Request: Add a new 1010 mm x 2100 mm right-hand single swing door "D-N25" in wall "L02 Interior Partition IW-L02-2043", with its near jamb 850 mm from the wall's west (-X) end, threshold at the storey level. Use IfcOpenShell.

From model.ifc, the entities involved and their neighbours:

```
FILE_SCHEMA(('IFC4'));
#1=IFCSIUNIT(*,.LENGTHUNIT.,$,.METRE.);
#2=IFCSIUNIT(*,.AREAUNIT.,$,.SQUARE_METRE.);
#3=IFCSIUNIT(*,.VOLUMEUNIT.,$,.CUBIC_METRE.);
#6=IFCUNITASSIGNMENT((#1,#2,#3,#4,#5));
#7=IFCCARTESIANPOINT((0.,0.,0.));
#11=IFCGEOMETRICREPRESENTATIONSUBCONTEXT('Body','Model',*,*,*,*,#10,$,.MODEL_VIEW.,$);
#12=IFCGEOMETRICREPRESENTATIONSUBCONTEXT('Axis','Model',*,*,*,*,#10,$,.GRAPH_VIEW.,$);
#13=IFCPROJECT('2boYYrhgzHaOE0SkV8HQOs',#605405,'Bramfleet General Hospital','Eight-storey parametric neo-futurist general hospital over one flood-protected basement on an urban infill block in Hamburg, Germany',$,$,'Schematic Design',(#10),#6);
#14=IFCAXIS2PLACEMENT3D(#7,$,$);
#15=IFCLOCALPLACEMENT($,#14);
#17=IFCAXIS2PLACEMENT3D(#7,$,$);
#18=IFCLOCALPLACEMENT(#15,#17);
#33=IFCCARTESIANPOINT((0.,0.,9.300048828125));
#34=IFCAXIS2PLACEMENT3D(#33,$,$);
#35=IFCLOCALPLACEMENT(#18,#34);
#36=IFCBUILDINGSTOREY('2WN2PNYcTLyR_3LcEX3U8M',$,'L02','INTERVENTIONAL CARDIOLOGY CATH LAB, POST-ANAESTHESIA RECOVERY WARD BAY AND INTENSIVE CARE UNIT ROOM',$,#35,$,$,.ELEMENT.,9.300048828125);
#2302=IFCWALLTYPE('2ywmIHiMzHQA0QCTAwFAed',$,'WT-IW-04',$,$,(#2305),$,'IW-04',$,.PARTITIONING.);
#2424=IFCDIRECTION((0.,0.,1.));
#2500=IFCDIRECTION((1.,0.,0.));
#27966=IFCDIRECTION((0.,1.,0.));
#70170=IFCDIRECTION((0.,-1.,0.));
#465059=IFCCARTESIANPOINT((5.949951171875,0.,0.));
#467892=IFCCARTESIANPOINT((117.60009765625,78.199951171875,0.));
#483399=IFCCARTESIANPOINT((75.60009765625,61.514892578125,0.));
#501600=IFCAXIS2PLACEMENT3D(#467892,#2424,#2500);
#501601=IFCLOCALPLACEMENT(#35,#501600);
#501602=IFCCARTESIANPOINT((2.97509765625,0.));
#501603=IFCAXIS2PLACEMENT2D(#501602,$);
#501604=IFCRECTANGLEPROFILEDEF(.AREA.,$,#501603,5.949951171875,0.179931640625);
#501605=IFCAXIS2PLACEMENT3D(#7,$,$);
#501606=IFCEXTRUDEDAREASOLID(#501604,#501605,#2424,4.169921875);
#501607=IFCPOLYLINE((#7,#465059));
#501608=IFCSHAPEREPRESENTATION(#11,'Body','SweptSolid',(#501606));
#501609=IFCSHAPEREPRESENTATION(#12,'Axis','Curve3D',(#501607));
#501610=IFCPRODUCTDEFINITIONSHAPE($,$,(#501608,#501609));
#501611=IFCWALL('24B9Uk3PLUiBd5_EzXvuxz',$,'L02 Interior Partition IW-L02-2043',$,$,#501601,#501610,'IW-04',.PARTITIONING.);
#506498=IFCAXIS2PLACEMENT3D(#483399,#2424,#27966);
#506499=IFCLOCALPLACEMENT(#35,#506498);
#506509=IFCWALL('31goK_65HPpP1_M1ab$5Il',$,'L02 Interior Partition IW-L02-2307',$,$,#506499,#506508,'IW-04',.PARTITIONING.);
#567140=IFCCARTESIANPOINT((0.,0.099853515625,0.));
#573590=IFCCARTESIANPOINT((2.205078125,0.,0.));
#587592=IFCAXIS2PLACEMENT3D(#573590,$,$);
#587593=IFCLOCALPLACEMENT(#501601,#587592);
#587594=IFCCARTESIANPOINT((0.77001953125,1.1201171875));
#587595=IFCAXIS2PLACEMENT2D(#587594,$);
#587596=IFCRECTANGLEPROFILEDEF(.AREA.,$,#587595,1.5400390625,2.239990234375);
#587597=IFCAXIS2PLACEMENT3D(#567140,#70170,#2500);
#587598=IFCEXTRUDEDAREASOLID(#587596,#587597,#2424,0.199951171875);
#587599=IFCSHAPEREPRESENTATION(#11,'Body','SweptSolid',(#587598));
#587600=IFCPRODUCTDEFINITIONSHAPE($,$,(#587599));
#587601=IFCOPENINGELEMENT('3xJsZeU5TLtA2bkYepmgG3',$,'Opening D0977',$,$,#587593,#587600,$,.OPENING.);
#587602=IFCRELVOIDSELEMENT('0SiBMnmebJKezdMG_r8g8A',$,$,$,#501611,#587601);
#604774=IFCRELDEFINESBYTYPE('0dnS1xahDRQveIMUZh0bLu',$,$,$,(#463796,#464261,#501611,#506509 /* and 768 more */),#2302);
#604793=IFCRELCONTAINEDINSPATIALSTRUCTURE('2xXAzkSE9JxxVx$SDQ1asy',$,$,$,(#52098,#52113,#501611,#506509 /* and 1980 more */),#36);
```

```python
import numpy as np
import ifcopenshell
import ifcopenshell.api.feature
import ifcopenshell.api.geometry
import ifcopenshell.api.root
import ifcopenshell.api.spatial
import ifcopenshell.geom
import ifcopenshell.util.element
import ifcopenshell.util.placement
import ifcopenshell.util.representation
import ifcopenshell.util.shape
import ifcopenshell.util.unit

model = ifcopenshell.open("model.ifc")
unit_scale = ifcopenshell.util.unit.calculate_unit_scale(model)
settings = ifcopenshell.geom.settings()


def volume(element):
    """Net volume in cubic metres, openings subtracted."""
    shape = ifcopenshell.geom.create_shape(settings, element)
    return ifcopenshell.util.shape.get_volume(shape.geometry)


wall = model.by_id(501611)
storey = ifcopenshell.util.element.get_container(wall, ifc_class="IfcBuildingStorey")
context = ifcopenshell.util.representation.get_context(model, "Model", "Body", "MODEL_VIEW")
before = volume(wall)

width, height, from_end, sill = 1.01, 2.1, 0.85, 0.0  # metres

# The wall runs along its own X axis, and the end named is its -X end.
wall_shape = ifcopenshell.geom.create_shape(settings, wall)
x, y, z = ifcopenshell.util.shape.get_vertices(wall_shape.geometry).T
start = x.min() + from_end
face, thickness = float(y.min()), float(y.max() - y.min())
wall_matrix = ifcopenshell.util.placement.get_local_placement(wall.ObjectPlacement)
level = ifcopenshell.util.placement.get_local_placement(storey.ObjectPlacement)[2, 3]


def in_wall(x, y):
    """Placement at x, y metres in the wall's axes, at sill height."""
    matrix = wall_matrix.copy()
    matrix[:, 3] = wall_matrix @ np.array([x / unit_scale, y / unit_scale, 0.0, 1.0])
    matrix[2, 3] = level + sill / unit_scale
    return matrix


# Opening: a box that overshoots both wall faces by 50 mm.
opening = ifcopenshell.api.root.create_entity(model, ifc_class="IfcOpeningElement", predefined_type="OPENING")
box = ifcopenshell.api.geometry.add_wall_representation(
    model, context=context, length=width, height=height, thickness=thickness + 0.1
)
ifcopenshell.api.geometry.assign_representation(model, product=opening, representation=box)
ifcopenshell.api.geometry.edit_object_placement(model, product=opening, matrix=in_wall(start, face - 0.05), is_si=False)
ifcopenshell.api.feature.add_feature(model, feature=opening, element=wall)

door = ifcopenshell.api.root.create_entity(model, ifc_class="IfcDoor", name="D-N25", predefined_type="DOOR")
door.OverallWidth, door.OverallHeight = width / unit_scale, height / unit_scale
door.OperationType = "SINGLE_SWING_RIGHT"
body = ifcopenshell.api.geometry.add_door_representation(
    model,
    context=context,
    overall_width=door.OverallWidth,
    overall_height=door.OverallHeight,
    operation_type="SINGLE_SWING_RIGHT",
    lining_properties={"LiningDepth": thickness / unit_scale, "ThresholdDepth": thickness / unit_scale},
)
ifcopenshell.api.geometry.assign_representation(model, product=door, representation=body)
ifcopenshell.api.spatial.assign_container(model, products=[door], relating_structure=storey)
ifcopenshell.api.feature.add_filling(model, opening=opening, element=door)

# The lining spans the wall, so the door starts at the wall face.
ifcopenshell.api.geometry.edit_object_placement(model, product=door, matrix=in_wall(start, face), is_si=False)

after = volume(wall)

print(f"wall volume {before:.3f} -> {after:.3f} m3")

model.write("model_rev.ifc")
```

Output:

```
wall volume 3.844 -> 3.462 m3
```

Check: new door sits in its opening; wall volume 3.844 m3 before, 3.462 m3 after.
